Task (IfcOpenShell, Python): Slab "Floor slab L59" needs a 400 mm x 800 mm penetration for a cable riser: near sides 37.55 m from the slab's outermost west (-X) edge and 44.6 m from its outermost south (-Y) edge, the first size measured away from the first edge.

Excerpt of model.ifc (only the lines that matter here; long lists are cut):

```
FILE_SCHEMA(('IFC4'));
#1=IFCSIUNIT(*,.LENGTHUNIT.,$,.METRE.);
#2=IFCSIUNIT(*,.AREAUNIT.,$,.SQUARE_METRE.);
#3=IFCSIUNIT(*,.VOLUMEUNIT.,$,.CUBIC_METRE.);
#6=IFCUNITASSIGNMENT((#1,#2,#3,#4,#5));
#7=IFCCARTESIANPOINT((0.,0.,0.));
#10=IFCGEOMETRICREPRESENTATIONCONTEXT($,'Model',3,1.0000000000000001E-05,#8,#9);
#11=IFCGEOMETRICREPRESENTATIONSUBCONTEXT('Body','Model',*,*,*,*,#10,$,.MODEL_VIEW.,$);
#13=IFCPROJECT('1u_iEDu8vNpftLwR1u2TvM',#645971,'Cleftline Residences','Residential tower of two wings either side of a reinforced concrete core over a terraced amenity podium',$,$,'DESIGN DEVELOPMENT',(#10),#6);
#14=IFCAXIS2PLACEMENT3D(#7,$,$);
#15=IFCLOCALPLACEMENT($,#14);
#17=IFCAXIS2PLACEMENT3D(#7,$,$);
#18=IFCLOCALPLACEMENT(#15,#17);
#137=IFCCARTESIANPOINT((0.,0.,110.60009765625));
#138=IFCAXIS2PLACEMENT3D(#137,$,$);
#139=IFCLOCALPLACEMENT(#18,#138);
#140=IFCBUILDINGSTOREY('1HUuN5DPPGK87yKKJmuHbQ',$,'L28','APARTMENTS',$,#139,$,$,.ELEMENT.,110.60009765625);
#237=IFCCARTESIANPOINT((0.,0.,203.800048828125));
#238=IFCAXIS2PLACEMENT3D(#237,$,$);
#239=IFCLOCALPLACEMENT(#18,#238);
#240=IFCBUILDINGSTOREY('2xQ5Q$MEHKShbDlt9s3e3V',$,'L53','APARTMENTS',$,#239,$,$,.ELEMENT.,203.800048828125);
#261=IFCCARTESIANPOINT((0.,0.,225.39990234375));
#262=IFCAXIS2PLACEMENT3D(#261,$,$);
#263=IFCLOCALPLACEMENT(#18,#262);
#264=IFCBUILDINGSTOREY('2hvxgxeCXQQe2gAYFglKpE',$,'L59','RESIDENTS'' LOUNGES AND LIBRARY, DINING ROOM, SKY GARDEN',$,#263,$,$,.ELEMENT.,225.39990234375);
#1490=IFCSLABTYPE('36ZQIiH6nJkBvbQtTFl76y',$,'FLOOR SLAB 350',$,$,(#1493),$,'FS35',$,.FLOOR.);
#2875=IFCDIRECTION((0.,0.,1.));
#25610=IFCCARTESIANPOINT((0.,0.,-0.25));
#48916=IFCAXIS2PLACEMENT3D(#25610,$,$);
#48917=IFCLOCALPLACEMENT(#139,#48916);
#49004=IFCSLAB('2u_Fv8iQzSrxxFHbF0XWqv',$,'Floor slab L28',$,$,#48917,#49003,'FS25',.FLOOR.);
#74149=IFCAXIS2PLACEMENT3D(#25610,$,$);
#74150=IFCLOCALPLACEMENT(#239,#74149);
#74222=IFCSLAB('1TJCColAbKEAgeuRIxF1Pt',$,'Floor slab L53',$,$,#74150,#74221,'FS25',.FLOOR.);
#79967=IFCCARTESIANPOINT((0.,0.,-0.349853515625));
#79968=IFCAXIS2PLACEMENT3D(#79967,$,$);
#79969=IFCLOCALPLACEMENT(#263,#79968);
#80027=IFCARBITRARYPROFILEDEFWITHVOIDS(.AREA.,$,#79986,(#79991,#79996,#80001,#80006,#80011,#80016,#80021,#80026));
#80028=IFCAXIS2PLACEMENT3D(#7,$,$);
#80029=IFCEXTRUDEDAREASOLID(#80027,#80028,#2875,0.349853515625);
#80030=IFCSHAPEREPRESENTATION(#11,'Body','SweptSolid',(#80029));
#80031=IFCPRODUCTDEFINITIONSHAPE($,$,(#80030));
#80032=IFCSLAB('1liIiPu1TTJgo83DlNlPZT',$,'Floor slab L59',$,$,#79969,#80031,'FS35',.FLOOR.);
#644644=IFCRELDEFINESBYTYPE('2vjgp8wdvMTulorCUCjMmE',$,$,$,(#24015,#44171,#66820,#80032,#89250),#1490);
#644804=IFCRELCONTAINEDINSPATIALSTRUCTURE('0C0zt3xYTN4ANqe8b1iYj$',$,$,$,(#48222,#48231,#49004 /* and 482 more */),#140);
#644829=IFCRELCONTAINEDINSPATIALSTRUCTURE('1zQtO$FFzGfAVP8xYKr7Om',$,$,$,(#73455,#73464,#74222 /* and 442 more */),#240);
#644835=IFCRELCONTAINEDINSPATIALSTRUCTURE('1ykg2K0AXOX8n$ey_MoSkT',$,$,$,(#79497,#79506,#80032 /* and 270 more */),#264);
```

```python
import numpy as np
import ifcopenshell
import ifcopenshell.api.feature
import ifcopenshell.api.geometry
import ifcopenshell.api.root
import ifcopenshell.geom
import ifcopenshell.util.placement
import ifcopenshell.util.representation
import ifcopenshell.util.shape
import ifcopenshell.util.unit

model = ifcopenshell.open("model.ifc")
unit_scale = ifcopenshell.util.unit.calculate_unit_scale(model)
settings = ifcopenshell.geom.settings()


def volume(element):
    """Net volume in cubic metres, openings subtracted."""
    shape = ifcopenshell.geom.create_shape(settings, element)
    return ifcopenshell.util.shape.get_volume(shape.geometry)


slab = model.by_id(80032)
before = volume(slab)

# Extent in the slab's own axes, in metres. The edges named are its -X and -Y sides.
slab_shape = ifcopenshell.geom.create_shape(settings, slab)
vertices = ifcopenshell.util.shape.get_vertices(slab_shape.geometry)
x_min, y_min, bottom = vertices.min(axis=0)
top = vertices[:, 2].max()

opening = ifcopenshell.api.root.create_entity(model, ifc_class="IfcOpeningElement", name="Cable riser opening", predefined_type="OPENING")
context = ifcopenshell.util.representation.get_context(model, "Model", "Body", "MODEL_VIEW")
width, depth = 0.4, 0.8
outline = [(0.0, 0.0), (width, 0.0), (width, depth), (0.0, depth), (0.0, 0.0)]
# Overshoot both faces by 50 mm so the cut is clean.
shape = ifcopenshell.api.geometry.add_slab_representation(
    model, context=context, depth=top - bottom + 0.1, polyline=outline
)
ifcopenshell.api.geometry.assign_representation(model, product=opening, representation=shape)

matrix = ifcopenshell.util.placement.get_local_placement(slab.ObjectPlacement)
matrix[:, 3] = matrix @ np.append(np.array([x_min + 37.55, y_min + 44.6, bottom - 0.05]) / unit_scale, 1.0)
ifcopenshell.api.geometry.edit_object_placement(model, product=opening, matrix=matrix, is_si=False)
ifcopenshell.api.feature.add_feature(model, feature=opening, element=slab)

after = volume(slab)

print(f"slab volume {before:.3f} -> {after:.3f} m3")

model.write("model-out.ifc")
```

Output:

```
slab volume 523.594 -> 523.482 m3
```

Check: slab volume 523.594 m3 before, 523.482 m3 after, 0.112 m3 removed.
